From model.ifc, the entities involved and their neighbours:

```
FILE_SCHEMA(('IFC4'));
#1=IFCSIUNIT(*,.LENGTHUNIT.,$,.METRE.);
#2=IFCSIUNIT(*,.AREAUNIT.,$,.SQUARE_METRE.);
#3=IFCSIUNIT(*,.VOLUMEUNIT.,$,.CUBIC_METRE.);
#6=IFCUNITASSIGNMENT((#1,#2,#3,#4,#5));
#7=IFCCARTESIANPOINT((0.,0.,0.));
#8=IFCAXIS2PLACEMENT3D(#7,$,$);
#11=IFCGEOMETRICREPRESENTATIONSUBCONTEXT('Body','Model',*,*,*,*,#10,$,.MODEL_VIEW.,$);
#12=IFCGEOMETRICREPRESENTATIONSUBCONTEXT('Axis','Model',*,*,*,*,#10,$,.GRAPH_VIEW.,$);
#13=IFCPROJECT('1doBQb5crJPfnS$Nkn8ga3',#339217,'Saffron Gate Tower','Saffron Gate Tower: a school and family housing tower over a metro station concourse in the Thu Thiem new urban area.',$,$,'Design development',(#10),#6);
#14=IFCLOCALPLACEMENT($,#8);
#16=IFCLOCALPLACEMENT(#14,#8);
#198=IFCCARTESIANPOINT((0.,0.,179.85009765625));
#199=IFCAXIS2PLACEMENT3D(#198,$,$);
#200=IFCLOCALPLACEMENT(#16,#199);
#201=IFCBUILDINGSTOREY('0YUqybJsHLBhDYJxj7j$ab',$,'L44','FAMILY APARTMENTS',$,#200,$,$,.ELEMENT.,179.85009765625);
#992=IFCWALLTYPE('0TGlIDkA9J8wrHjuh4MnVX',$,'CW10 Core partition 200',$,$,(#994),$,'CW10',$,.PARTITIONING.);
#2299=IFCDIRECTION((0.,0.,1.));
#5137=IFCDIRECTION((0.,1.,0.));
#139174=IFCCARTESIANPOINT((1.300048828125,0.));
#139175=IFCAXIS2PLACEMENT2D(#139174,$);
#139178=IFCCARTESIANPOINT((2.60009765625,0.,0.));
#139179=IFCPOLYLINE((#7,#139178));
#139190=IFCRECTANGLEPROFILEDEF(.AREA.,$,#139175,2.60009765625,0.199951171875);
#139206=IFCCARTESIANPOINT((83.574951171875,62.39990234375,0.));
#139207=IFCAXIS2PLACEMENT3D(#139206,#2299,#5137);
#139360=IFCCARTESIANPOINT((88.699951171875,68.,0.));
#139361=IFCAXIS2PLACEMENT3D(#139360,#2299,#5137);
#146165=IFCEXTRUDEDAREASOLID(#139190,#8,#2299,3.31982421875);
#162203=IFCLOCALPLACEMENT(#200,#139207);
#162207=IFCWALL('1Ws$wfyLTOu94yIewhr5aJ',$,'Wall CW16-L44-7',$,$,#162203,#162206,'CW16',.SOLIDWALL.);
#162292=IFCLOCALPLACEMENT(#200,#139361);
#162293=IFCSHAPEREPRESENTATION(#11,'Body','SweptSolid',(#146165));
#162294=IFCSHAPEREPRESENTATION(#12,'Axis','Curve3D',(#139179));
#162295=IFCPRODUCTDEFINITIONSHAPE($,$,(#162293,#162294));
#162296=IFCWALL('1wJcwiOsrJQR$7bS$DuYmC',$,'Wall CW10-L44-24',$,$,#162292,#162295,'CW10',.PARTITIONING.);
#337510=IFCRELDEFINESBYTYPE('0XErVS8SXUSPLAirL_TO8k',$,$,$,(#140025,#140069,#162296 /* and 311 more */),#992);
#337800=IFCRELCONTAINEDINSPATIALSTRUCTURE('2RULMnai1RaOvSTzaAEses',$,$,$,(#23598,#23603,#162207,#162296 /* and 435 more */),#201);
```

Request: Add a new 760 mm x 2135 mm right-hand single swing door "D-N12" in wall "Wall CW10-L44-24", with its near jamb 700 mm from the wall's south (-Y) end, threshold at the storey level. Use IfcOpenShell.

```python
import numpy as np
import ifcopenshell
import ifcopenshell.api.feature
import ifcopenshell.api.geometry
import ifcopenshell.api.root
import ifcopenshell.api.spatial
import ifcopenshell.geom
import ifcopenshell.util.element
import ifcopenshell.util.placement
import ifcopenshell.util.representation
import ifcopenshell.util.shape
import ifcopenshell.util.unit

model = ifcopenshell.open("model.ifc")
unit_scale = ifcopenshell.util.unit.calculate_unit_scale(model)
settings = ifcopenshell.geom.settings()


def volume(element):
    """Net volume in cubic metres, openings subtracted."""
    shape = ifcopenshell.geom.create_shape(settings, element)
    return ifcopenshell.util.shape.get_volume(shape.geometry)


wall = model.by_guid("1wJcwiOsrJQR$7bS$DuYmC")
storey = ifcopenshell.util.element.get_container(wall, ifc_class="IfcBuildingStorey")
context = ifcopenshell.util.representation.get_context(model, "Model", "Body", "MODEL_VIEW")
before = volume(wall)

width, height, from_end, sill = 0.76, 2.135, 0.7, 0.0  # metres

# The wall runs along its own X axis, and the end named is its -X end.
wall_shape = ifcopenshell.geom.create_shape(settings, wall)
x, y, z = ifcopenshell.util.shape.get_vertices(wall_shape.geometry).T
start = x.min() + from_end
face, thickness = float(y.min()), float(y.max() - y.min())
wall_matrix = ifcopenshell.util.placement.get_local_placement(wall.ObjectPlacement)
level = ifcopenshell.util.placement.get_local_placement(storey.ObjectPlacement)[2, 3]


def in_wall(x, y):
    """Placement at x, y metres in the wall's axes, at sill height."""
    matrix = wall_matrix.copy()
    matrix[:, 3] = wall_matrix @ np.array([x / unit_scale, y / unit_scale, 0.0, 1.0])
    matrix[2, 3] = level + sill / unit_scale
    return matrix


# Opening: a box that overshoots both wall faces by 50 mm.
opening = ifcopenshell.api.root.create_entity(model, ifc_class="IfcOpeningElement", predefined_type="OPENING")
box = ifcopenshell.api.geometry.add_wall_representation(
    model, context=context, length=width, height=height, thickness=thickness + 0.1
)
ifcopenshell.api.geometry.assign_representation(model, product=opening, representation=box)
ifcopenshell.api.geometry.edit_object_placement(model, product=opening, matrix=in_wall(start, face - 0.05), is_si=False)
ifcopenshell.api.feature.add_feature(model, feature=opening, element=wall)

door = ifcopenshell.api.root.create_entity(model, ifc_class="IfcDoor", name="D-N12", predefined_type="DOOR")
door.OverallWidth, door.OverallHeight = width / unit_scale, height / unit_scale
door.OperationType = "SINGLE_SWING_RIGHT"
body = ifcopenshell.api.geometry.add_door_representation(
    model,
    context=context,
    overall_width=door.OverallWidth,
    overall_height=door.OverallHeight,
    operation_type="SINGLE_SWING_RIGHT",
    lining_properties={"LiningDepth": thickness / unit_scale, "ThresholdDepth": thickness / unit_scale},
)
ifcopenshell.api.geometry.assign_representation(model, product=door, representation=body)
ifcopenshell.api.spatial.assign_container(model, products=[door], relating_structure=storey)
ifcopenshell.api.feature.add_filling(model, opening=opening, element=door)

# The lining spans the wall, so the door starts at the wall face.
ifcopenshell.api.geometry.edit_object_placement(model, product=door, matrix=in_wall(start, face), is_si=False)

after = volume(wall)

print(f"wall volume {before:.3f} -> {after:.3f} m3")

model.write("model_v2.ifc")
```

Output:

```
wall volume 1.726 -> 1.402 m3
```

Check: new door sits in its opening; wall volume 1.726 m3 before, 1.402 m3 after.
